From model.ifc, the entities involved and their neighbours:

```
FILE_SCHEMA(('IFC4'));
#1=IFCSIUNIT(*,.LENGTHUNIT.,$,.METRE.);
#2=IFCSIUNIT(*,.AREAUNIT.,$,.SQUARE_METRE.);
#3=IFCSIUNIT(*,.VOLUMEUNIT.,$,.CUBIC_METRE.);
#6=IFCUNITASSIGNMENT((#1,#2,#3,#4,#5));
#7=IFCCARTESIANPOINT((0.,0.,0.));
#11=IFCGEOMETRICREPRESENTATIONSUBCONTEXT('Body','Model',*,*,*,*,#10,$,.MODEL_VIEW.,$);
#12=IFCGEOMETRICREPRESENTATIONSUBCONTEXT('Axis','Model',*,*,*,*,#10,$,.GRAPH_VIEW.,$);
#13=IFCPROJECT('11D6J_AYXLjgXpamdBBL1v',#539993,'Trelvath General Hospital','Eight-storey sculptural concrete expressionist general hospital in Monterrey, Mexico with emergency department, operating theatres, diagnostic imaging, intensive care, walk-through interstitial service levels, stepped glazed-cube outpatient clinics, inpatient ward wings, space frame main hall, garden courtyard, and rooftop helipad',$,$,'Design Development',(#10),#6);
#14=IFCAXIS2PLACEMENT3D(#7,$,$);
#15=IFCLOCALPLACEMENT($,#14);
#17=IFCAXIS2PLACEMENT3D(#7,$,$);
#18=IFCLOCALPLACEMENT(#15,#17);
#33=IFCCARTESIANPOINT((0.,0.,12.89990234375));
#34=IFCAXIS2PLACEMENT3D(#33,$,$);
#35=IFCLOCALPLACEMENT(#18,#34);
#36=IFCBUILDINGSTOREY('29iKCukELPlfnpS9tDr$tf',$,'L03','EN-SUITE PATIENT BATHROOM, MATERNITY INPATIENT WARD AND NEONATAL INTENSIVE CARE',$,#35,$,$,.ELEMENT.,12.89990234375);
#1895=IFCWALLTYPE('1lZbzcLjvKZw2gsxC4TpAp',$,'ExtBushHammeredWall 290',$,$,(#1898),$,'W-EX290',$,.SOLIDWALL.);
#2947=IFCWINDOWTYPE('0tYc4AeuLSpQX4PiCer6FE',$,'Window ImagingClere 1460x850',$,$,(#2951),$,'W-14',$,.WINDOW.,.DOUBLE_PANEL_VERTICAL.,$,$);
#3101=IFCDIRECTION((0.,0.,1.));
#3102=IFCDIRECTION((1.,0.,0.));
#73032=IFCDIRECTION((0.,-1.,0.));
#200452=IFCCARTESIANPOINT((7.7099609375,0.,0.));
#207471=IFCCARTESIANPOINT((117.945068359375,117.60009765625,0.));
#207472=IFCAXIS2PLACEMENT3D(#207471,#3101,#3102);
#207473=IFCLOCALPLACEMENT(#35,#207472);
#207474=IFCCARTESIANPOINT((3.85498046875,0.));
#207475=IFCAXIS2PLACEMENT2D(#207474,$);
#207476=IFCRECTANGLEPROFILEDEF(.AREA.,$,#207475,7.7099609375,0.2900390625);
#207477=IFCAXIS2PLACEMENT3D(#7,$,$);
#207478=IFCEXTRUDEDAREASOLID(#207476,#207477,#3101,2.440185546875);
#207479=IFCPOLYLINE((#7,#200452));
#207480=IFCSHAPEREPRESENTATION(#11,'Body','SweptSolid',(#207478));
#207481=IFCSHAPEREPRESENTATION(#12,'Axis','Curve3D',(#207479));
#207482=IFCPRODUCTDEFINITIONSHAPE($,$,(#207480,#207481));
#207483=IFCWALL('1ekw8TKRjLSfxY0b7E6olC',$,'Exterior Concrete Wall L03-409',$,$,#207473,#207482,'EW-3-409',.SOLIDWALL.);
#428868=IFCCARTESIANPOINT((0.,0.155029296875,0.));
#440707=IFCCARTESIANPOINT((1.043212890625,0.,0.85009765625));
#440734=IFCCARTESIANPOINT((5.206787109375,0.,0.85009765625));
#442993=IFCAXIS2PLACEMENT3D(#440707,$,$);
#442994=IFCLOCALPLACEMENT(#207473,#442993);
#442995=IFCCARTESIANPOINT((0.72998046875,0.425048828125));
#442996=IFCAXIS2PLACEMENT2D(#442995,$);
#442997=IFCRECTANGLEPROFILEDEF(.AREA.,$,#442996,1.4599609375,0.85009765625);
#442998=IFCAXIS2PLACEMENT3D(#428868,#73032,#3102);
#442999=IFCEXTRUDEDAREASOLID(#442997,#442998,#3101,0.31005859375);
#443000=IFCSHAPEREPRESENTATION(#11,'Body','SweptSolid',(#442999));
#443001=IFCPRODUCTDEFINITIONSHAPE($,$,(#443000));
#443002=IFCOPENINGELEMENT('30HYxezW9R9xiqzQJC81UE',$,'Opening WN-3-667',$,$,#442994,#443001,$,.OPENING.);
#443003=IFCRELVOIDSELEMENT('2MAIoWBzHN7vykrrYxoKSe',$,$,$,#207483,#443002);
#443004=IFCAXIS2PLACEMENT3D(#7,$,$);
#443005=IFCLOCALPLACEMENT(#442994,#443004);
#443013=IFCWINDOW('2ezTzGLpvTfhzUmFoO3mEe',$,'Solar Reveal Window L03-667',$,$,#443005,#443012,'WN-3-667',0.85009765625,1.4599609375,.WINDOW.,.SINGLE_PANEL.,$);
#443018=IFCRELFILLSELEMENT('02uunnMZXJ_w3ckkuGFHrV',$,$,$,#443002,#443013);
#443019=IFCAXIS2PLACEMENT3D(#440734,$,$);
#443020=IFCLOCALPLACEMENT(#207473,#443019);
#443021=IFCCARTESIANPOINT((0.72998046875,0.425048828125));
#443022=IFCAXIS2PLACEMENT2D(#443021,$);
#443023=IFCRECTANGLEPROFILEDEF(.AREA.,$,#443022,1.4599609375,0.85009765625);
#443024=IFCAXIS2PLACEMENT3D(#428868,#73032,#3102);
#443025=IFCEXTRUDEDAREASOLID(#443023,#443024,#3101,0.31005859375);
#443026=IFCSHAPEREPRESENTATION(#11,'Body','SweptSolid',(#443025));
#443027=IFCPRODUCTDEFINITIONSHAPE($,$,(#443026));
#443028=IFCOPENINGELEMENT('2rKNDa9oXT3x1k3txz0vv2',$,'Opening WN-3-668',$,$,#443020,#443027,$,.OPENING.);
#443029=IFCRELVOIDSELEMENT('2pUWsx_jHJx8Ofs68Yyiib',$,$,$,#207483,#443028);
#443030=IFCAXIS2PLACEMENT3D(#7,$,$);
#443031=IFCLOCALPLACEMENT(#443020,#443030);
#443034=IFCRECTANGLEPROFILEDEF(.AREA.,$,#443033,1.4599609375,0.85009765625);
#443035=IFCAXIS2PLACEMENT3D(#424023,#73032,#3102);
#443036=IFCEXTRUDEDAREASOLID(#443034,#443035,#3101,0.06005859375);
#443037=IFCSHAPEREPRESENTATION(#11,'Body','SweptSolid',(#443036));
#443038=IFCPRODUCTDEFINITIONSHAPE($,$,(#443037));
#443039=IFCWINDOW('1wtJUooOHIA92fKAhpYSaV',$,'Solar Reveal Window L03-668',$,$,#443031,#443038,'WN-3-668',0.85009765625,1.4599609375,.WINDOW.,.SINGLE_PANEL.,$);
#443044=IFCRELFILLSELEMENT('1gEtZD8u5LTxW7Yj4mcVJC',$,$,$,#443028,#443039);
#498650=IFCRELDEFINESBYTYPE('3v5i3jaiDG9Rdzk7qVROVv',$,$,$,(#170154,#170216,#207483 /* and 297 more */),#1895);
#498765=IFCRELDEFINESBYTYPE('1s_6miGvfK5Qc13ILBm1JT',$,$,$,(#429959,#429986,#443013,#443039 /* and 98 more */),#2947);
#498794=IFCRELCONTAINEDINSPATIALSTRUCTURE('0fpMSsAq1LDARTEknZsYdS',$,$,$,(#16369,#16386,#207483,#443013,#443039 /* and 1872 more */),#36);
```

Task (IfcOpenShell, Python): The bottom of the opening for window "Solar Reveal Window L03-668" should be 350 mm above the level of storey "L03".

```python
import numpy as np
import ifcopenshell
import ifcopenshell.api.geometry
import ifcopenshell.geom
import ifcopenshell.util.element
import ifcopenshell.util.placement
import ifcopenshell.util.shape
import ifcopenshell.util.unit

model = ifcopenshell.open("model.ifc")
unit_scale = ifcopenshell.util.unit.calculate_unit_scale(model)

window = model.by_id(443039)
opening = window.FillsVoids[0].RelatingOpeningElement
storey = ifcopenshell.util.element.get_container(window, ifc_class="IfcBuildingStorey")
level = ifcopenshell.util.placement.get_local_placement(storey.ObjectPlacement)[2, 3]

# The opening's origin need not be at the sill, so measure its lowest point.
shape = ifcopenshell.geom.create_shape(ifcopenshell.geom.settings(), opening)
bottom = ifcopenshell.util.shape.get_shape_bottom_elevation(shape, shape.geometry) / unit_scale
dz = level + 0.35 - bottom

shift = np.array([0.0, 0.0, dz])
# The window is placed relative to its opening, so it follows when the opening moves.
matrix = ifcopenshell.util.placement.get_local_placement(opening.ObjectPlacement)
matrix[:3, 3] += shift
ifcopenshell.api.geometry.edit_object_placement(
    model, product=opening, matrix=matrix, is_si=False, should_transform_children=True
)

print(f"moved by {dz * unit_scale:+.3f} m")

model.write("model_v2.ifc")
```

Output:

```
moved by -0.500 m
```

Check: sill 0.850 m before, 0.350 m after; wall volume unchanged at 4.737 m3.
